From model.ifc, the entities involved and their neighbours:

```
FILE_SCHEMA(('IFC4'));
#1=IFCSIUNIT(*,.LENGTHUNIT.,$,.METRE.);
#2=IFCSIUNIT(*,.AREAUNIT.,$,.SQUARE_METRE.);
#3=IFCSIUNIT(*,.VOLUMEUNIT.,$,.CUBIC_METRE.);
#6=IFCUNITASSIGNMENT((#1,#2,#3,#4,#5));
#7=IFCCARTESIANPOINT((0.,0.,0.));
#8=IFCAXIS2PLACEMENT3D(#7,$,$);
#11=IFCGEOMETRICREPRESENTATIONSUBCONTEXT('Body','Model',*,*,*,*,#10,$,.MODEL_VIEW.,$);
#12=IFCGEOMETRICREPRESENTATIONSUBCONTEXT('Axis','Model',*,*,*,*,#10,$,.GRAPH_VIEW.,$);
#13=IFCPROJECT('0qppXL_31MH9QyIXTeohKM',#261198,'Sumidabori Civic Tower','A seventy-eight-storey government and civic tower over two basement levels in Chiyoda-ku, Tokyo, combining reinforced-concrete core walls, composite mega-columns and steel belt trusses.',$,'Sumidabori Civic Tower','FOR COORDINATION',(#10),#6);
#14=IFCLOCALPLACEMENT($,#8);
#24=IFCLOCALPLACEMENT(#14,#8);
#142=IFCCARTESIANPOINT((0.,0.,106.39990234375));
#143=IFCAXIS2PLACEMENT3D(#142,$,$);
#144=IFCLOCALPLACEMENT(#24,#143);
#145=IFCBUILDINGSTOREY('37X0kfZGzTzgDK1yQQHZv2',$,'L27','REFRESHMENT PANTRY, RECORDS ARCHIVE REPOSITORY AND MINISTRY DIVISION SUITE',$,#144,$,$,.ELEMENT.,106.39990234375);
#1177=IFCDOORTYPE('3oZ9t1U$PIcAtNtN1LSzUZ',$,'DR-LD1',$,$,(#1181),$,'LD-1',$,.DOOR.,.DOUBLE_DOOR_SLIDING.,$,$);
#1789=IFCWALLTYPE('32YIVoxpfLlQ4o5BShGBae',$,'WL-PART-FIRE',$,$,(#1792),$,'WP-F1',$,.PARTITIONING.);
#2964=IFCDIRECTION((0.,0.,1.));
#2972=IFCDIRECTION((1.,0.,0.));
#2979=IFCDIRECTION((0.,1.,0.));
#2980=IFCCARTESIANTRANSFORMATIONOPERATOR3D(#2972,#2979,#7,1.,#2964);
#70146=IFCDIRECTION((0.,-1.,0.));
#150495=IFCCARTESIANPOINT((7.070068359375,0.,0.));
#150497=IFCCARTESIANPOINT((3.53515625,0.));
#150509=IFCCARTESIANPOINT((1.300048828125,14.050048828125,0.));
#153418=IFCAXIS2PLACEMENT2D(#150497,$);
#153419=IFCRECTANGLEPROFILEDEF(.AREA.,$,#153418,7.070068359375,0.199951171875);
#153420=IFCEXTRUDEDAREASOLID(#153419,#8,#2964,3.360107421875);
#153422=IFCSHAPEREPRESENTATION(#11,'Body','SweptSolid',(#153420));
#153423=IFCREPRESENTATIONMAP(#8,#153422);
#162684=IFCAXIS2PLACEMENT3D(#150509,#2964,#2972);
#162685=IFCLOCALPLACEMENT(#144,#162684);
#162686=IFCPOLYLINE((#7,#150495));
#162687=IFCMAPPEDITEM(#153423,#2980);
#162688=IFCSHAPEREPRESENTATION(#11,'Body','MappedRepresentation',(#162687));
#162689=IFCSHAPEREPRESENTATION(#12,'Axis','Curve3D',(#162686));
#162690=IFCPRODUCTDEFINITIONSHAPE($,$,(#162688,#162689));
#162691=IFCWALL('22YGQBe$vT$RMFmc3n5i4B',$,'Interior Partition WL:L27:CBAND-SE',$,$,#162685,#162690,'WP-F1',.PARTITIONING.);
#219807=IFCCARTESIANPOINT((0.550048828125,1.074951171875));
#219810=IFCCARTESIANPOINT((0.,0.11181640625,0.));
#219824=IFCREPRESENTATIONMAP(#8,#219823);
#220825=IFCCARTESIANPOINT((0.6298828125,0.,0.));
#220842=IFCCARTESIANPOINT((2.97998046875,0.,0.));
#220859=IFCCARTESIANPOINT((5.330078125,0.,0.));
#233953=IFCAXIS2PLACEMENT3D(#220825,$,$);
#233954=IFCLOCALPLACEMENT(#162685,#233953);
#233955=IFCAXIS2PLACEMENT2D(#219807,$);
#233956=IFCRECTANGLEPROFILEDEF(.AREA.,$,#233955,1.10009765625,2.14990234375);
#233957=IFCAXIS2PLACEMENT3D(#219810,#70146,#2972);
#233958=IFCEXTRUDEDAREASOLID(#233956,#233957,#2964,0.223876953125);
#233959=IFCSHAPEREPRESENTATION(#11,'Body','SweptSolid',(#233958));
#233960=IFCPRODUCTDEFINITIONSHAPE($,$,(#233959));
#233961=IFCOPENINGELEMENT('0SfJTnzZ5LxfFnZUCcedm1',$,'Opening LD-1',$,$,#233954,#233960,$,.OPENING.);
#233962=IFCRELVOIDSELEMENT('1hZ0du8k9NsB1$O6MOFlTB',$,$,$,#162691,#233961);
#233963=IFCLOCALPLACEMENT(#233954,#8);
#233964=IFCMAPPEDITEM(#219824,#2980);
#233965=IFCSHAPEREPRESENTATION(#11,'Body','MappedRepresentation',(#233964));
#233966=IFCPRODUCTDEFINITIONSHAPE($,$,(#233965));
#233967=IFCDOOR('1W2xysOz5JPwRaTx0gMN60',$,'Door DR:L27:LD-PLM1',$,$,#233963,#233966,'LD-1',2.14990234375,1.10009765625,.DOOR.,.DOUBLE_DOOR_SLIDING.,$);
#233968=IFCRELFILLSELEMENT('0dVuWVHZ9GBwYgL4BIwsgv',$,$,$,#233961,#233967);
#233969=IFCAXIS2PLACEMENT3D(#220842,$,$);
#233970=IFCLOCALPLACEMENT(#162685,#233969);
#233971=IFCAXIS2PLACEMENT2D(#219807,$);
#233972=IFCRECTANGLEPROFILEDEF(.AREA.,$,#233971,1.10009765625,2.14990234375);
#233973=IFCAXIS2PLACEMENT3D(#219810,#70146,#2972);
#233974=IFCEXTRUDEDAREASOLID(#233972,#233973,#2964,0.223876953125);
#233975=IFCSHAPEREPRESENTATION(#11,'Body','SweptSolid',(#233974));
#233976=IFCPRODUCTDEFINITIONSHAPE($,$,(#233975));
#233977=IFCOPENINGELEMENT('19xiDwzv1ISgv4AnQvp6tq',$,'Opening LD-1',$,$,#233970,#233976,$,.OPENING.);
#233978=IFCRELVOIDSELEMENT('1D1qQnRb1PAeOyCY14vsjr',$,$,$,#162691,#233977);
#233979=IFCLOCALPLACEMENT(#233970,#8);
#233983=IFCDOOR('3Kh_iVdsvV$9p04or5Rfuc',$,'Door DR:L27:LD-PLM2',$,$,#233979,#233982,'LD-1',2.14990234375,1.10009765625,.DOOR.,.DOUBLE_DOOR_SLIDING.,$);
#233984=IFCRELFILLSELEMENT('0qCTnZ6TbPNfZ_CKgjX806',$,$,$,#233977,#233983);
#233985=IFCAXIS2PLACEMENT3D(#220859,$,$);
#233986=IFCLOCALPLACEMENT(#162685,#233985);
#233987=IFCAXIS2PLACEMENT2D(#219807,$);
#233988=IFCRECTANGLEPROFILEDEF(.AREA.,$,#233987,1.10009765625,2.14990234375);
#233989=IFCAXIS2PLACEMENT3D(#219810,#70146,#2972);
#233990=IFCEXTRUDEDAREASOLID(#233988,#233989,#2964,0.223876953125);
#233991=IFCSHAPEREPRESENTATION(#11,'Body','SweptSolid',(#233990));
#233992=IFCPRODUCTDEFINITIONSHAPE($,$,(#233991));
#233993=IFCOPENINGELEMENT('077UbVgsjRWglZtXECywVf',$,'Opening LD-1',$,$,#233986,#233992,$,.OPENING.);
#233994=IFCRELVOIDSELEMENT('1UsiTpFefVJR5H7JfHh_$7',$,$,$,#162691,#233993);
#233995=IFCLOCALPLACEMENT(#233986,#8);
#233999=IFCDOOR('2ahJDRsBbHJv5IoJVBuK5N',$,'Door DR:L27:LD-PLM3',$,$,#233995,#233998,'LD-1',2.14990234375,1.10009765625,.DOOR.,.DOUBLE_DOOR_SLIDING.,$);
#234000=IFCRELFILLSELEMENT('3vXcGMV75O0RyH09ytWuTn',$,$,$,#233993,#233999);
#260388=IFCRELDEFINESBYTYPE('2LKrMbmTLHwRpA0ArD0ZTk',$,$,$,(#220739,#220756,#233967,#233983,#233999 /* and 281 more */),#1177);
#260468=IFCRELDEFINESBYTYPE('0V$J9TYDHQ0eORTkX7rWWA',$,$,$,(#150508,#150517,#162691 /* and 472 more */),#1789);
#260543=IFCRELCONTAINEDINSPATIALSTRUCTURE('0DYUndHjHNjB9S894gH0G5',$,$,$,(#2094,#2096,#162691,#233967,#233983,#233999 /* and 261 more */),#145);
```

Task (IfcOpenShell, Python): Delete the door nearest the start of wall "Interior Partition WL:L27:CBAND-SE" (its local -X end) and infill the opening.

```python
import ifcopenshell
import ifcopenshell.api.feature
import ifcopenshell.api.root
import ifcopenshell.geom
import ifcopenshell.util.shape

model = ifcopenshell.open("model.ifc")
settings = ifcopenshell.geom.settings()


def volume(element):
    """Net volume in cubic metres, openings subtracted."""
    shape = ifcopenshell.geom.create_shape(settings, element)
    return ifcopenshell.util.shape.get_volume(shape.geometry)


door = model.by_guid("1W2xysOz5JPwRaTx0gMN60")
opening = door.FillsVoids[0].RelatingOpeningElement
wall = opening.VoidsElements[0].RelatingBuildingElement
before = volume(wall)

ifcopenshell.api.root.remove_product(model, product=door)
ifcopenshell.api.feature.remove_feature(model, feature=opening)

after = volume(wall)

print(f"wall volume {before:.3f} -> {after:.3f} m3")

model.write("model_edited.ifc")
```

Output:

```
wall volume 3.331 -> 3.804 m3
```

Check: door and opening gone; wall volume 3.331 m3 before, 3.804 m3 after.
